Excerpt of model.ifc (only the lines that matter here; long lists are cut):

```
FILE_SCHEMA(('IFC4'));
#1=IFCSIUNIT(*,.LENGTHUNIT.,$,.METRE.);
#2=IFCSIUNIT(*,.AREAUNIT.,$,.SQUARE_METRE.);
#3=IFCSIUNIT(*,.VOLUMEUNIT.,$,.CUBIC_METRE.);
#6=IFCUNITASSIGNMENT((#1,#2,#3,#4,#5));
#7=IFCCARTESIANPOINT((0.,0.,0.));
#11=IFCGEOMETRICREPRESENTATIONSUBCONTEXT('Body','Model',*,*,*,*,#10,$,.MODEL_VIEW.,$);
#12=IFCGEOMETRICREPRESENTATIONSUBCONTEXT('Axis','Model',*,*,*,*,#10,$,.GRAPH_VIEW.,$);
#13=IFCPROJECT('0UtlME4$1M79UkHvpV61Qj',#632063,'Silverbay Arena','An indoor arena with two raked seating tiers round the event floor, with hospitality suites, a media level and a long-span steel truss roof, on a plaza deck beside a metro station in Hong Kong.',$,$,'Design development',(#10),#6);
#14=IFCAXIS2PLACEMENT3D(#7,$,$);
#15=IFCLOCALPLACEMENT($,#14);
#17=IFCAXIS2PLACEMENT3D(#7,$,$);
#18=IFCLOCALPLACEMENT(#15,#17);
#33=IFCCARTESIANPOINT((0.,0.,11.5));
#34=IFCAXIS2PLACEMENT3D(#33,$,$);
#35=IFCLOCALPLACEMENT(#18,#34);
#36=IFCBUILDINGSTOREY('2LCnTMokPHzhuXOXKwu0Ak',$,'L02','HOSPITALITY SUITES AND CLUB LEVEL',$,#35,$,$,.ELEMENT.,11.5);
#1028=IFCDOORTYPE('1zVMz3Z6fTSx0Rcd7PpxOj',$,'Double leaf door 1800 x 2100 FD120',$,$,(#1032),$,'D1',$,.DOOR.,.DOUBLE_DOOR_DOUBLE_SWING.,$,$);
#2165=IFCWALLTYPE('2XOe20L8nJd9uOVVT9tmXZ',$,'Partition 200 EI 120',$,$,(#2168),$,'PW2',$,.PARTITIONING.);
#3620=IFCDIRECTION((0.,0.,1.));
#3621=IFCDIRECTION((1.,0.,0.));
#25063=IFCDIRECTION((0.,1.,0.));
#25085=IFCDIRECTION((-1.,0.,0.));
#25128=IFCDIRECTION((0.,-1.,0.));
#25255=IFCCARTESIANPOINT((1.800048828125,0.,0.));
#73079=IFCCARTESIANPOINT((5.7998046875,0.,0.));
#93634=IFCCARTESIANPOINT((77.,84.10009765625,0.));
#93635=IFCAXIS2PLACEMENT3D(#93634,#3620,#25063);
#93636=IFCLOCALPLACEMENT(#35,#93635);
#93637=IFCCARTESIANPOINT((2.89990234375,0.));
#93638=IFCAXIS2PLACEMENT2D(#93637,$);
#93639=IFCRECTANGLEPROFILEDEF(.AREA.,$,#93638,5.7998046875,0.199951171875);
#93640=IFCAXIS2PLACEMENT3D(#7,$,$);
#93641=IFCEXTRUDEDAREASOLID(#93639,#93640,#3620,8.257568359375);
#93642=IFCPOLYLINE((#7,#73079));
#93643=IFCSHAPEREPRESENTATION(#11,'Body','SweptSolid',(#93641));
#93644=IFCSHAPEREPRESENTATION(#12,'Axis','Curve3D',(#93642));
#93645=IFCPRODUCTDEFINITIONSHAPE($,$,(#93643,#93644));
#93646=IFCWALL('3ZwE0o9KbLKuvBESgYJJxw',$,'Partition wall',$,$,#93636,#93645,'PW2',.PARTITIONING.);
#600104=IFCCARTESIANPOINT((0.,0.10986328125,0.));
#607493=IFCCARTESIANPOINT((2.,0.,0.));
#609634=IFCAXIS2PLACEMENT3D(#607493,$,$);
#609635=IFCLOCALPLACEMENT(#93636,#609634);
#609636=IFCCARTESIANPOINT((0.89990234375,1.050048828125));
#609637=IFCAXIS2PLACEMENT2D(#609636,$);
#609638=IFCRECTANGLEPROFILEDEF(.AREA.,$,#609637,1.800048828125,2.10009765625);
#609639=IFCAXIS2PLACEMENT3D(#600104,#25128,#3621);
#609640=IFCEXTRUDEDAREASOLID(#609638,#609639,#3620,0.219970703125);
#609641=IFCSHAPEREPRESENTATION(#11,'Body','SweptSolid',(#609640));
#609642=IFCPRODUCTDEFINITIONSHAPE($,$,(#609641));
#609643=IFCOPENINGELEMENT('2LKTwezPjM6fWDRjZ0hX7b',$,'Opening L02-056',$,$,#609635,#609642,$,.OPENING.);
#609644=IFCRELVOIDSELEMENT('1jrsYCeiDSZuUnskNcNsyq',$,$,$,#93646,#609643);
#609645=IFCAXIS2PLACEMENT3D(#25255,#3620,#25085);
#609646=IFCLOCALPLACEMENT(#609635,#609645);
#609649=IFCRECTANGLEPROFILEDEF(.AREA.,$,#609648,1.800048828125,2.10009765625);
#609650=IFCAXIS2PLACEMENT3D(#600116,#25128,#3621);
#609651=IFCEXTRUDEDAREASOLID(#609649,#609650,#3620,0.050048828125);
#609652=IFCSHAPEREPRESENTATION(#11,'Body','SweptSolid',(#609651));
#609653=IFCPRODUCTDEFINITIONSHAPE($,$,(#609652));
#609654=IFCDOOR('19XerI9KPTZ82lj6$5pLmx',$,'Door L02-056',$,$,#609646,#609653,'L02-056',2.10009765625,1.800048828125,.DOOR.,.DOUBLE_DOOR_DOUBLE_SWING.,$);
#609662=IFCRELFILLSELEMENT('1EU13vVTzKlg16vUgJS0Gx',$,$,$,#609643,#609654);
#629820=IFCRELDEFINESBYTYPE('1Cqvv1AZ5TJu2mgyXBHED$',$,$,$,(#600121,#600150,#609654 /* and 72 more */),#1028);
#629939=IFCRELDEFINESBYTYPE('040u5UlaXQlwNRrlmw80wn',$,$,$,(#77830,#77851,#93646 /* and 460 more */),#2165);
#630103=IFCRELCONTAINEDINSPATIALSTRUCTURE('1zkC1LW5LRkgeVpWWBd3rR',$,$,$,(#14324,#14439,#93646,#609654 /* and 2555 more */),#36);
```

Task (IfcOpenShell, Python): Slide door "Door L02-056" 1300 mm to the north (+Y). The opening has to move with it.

```python
import ifcopenshell
import ifcopenshell.api.geometry
import ifcopenshell.util.placement
import ifcopenshell.util.unit

model = ifcopenshell.open("model.ifc")
unit_scale = ifcopenshell.util.unit.calculate_unit_scale(model)

door = model.by_guid("19XerI9KPTZ82lj6$5pLmx")
opening = door.FillsVoids[0].RelatingOpeningElement
wall = opening.VoidsElements[0].RelatingBuildingElement

wall_matrix = ifcopenshell.util.placement.get_local_placement(wall.ObjectPlacement)
shift = wall_matrix[:3, 0] * 1.3 / unit_scale
before = ifcopenshell.util.placement.get_local_placement(door.ObjectPlacement)[:3, 3].copy()

# The door is placed relative to its opening, so it follows when the opening moves.
matrix = ifcopenshell.util.placement.get_local_placement(opening.ObjectPlacement)
matrix[:3, 3] += shift
ifcopenshell.api.geometry.edit_object_placement(
    model, product=opening, matrix=matrix, is_si=False, should_transform_children=True
)

after = ifcopenshell.util.placement.get_local_placement(door.ObjectPlacement)[:3, 3]
print("door moved by", (after - before).round(3) + 0.0)

model.write("model_v2.ifc")
```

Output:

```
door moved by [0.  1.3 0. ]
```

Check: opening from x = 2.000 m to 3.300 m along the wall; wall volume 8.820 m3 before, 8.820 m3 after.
